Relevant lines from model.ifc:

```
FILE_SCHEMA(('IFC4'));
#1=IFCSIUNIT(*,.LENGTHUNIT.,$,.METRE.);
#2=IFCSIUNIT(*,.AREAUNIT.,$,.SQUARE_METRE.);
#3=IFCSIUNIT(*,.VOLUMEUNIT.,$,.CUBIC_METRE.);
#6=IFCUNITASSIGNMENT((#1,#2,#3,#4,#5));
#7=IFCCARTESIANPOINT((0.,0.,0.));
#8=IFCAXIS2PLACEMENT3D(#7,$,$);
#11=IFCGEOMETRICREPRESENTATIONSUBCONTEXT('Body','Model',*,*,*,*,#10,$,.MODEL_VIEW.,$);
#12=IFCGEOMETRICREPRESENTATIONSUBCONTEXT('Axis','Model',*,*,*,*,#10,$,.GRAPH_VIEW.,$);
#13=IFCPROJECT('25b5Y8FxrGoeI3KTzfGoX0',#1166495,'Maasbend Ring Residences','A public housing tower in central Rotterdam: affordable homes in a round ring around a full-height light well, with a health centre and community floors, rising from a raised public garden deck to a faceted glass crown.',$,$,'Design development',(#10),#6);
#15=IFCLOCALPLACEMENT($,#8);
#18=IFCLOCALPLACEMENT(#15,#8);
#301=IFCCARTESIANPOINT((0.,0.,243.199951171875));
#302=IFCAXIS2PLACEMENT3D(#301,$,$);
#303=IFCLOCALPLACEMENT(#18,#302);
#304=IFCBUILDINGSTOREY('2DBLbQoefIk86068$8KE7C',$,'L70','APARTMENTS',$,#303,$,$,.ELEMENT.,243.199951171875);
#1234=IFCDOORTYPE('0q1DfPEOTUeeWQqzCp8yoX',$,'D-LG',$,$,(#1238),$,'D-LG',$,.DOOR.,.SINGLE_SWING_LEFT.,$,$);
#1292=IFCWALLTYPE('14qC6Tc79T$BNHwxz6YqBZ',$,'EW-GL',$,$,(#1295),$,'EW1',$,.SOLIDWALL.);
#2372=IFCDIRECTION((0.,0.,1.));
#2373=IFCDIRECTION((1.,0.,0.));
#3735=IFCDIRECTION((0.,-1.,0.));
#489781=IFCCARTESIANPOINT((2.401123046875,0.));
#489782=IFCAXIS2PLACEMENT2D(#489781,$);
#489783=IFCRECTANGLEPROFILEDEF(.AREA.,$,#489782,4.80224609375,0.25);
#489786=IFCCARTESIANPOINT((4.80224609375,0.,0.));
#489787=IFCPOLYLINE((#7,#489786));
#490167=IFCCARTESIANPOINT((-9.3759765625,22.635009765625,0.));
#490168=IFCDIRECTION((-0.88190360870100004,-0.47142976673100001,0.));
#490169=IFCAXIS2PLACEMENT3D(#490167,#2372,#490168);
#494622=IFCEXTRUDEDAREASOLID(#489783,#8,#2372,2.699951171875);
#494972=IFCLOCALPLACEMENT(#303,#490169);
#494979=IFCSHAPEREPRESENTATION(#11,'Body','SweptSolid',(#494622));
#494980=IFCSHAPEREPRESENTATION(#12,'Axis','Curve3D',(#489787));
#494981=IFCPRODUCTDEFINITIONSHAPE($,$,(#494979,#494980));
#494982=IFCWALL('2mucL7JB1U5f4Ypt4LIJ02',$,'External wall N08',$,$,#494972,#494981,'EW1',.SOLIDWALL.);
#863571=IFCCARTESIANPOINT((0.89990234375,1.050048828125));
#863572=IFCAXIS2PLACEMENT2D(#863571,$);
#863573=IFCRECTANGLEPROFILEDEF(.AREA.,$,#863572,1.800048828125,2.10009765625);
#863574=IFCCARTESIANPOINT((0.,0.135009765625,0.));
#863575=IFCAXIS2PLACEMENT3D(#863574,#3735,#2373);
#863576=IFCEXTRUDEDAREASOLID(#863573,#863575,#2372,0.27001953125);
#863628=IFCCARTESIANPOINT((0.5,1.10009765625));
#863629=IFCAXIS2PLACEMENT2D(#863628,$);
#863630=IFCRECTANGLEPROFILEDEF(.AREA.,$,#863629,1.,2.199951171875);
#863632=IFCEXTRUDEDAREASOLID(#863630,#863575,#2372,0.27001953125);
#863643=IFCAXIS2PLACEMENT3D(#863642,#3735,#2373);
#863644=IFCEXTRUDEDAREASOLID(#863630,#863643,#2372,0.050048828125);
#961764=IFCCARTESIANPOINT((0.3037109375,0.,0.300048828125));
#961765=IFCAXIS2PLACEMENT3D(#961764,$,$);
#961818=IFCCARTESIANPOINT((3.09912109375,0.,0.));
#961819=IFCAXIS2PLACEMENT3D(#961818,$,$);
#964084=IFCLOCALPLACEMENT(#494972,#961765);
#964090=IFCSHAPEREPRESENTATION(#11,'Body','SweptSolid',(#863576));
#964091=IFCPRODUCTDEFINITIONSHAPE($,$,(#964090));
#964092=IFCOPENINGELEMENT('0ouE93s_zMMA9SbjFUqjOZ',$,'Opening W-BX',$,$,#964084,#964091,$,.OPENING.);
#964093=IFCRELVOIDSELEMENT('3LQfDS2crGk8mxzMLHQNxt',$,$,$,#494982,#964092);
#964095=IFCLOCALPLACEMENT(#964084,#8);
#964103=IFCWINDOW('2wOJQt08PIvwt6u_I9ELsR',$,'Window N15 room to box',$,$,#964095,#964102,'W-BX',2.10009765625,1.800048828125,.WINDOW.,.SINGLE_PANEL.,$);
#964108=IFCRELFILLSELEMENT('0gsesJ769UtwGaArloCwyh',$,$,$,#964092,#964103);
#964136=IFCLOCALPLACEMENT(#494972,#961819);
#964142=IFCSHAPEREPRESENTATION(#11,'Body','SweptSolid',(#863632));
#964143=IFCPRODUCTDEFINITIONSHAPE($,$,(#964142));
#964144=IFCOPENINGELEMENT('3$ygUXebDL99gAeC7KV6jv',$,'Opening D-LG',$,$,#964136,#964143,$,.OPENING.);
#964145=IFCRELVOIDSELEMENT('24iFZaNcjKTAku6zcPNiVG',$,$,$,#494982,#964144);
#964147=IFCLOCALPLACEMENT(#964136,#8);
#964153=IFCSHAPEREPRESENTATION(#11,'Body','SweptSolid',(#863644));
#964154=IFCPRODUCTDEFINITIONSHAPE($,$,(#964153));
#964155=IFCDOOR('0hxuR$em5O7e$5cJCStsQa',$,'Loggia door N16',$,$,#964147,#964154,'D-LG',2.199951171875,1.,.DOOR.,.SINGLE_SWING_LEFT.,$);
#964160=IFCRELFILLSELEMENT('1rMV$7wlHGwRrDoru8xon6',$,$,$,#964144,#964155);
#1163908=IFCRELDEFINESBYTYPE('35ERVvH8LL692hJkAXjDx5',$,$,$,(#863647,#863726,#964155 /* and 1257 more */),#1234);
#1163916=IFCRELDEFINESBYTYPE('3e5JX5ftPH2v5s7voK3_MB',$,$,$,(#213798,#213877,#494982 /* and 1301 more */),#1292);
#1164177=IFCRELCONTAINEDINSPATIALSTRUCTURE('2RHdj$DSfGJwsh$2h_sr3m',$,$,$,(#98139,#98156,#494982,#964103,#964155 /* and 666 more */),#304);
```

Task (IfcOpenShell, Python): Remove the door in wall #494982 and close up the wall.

```python
import ifcopenshell
import ifcopenshell.api.feature
import ifcopenshell.api.root
import ifcopenshell.geom
import ifcopenshell.util.shape

model = ifcopenshell.open("model.ifc")
settings = ifcopenshell.geom.settings()


def volume(element):
    """Net volume in cubic metres, openings subtracted."""
    shape = ifcopenshell.geom.create_shape(settings, element)
    return ifcopenshell.util.shape.get_volume(shape.geometry)


door = model.by_guid("0hxuR$em5O7e$5cJCStsQa")
opening = door.FillsVoids[0].RelatingOpeningElement
wall = opening.VoidsElements[0].RelatingBuildingElement
before = volume(wall)

ifcopenshell.api.root.remove_product(model, product=door)
ifcopenshell.api.feature.remove_feature(model, feature=opening)

after = volume(wall)

print(f"wall volume {before:.3f} -> {after:.3f} m3")

model.write("model-out.ifc")
```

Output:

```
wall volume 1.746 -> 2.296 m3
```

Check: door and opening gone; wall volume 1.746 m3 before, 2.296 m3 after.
